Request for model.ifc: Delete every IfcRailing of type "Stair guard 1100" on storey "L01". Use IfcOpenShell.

First a look at what the model holds.

```python
import ifcopenshell
import ifcopenshell.util.element

model = ifcopenshell.open("model.ifc")
print(model.schema)
storey = next(s for s in model.by_type("IfcBuildingStorey") if s.Name == "L01")
railings = [e for e in ifcopenshell.util.element.get_decomposition(storey) if e.is_a("IfcRailing")]
seen = {}
for e in railings:
    element_type = ifcopenshell.util.element.get_type(e)
    name = element_type.Name if element_type not in (None, e) else None
    seen[name] = seen.get(name, 0) + 1
for name, count in sorted(seen.items(), key=str):
    print(count, "x", name)
```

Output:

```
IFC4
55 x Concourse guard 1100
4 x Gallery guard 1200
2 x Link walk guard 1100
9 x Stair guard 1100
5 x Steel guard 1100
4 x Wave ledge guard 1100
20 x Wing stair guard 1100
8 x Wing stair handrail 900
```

```python
import ifcopenshell
import ifcopenshell.api.root
import ifcopenshell.util.element

model = ifcopenshell.open("model.ifc")

storey = next(s for s in model.by_type("IfcBuildingStorey") if s.Name == "L01")
railings = [e for e in ifcopenshell.util.element.get_decomposition(storey) if e.is_a("IfcRailing")]
targets = [e for e in railings if (t := ifcopenshell.util.element.get_type(e)) not in (None, e) and t.Name == "Stair guard 1100"]

for e in targets:
    ifcopenshell.api.root.remove_product(model, product=e)
print(len(targets), "removed")

model.write("model_edited.ifc")
```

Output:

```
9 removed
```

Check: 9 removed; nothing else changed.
